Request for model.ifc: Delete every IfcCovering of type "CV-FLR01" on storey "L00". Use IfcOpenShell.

First a look at what the model holds.

```python
import ifcopenshell
import ifcopenshell.util.element

model = ifcopenshell.open("model.ifc")
print(model.schema)
storey = next(s for s in model.by_type("IfcBuildingStorey") if s.Name == "L00")
coverings = [e for e in ifcopenshell.util.element.get_decomposition(storey) if e.is_a("IfcCovering")]
seen = {}
for e in coverings:
    element_type = ifcopenshell.util.element.get_type(e)
    name = element_type.Name if element_type not in (None, e) else None
    seen[name] = seen.get(name, 0) + 1
for name, count in sorted(seen.items(), key=str):
    print(count, "x", name)
```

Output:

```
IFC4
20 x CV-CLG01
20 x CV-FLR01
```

```python
import ifcopenshell
import ifcopenshell.api.root
import ifcopenshell.util.element

model = ifcopenshell.open("model.ifc")

storey = next(s for s in model.by_type("IfcBuildingStorey") if s.Name == "L00")
coverings = [e for e in ifcopenshell.util.element.get_decomposition(storey) if e.is_a("IfcCovering")]
targets = [e for e in coverings if (t := ifcopenshell.util.element.get_type(e)) not in (None, e) and t.Name == "CV-FLR01"]

for e in targets:
    ifcopenshell.api.root.remove_product(model, product=e)
print(len(targets), "removed")

model.write("model_rev.ifc")
```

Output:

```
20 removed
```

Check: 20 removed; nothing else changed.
